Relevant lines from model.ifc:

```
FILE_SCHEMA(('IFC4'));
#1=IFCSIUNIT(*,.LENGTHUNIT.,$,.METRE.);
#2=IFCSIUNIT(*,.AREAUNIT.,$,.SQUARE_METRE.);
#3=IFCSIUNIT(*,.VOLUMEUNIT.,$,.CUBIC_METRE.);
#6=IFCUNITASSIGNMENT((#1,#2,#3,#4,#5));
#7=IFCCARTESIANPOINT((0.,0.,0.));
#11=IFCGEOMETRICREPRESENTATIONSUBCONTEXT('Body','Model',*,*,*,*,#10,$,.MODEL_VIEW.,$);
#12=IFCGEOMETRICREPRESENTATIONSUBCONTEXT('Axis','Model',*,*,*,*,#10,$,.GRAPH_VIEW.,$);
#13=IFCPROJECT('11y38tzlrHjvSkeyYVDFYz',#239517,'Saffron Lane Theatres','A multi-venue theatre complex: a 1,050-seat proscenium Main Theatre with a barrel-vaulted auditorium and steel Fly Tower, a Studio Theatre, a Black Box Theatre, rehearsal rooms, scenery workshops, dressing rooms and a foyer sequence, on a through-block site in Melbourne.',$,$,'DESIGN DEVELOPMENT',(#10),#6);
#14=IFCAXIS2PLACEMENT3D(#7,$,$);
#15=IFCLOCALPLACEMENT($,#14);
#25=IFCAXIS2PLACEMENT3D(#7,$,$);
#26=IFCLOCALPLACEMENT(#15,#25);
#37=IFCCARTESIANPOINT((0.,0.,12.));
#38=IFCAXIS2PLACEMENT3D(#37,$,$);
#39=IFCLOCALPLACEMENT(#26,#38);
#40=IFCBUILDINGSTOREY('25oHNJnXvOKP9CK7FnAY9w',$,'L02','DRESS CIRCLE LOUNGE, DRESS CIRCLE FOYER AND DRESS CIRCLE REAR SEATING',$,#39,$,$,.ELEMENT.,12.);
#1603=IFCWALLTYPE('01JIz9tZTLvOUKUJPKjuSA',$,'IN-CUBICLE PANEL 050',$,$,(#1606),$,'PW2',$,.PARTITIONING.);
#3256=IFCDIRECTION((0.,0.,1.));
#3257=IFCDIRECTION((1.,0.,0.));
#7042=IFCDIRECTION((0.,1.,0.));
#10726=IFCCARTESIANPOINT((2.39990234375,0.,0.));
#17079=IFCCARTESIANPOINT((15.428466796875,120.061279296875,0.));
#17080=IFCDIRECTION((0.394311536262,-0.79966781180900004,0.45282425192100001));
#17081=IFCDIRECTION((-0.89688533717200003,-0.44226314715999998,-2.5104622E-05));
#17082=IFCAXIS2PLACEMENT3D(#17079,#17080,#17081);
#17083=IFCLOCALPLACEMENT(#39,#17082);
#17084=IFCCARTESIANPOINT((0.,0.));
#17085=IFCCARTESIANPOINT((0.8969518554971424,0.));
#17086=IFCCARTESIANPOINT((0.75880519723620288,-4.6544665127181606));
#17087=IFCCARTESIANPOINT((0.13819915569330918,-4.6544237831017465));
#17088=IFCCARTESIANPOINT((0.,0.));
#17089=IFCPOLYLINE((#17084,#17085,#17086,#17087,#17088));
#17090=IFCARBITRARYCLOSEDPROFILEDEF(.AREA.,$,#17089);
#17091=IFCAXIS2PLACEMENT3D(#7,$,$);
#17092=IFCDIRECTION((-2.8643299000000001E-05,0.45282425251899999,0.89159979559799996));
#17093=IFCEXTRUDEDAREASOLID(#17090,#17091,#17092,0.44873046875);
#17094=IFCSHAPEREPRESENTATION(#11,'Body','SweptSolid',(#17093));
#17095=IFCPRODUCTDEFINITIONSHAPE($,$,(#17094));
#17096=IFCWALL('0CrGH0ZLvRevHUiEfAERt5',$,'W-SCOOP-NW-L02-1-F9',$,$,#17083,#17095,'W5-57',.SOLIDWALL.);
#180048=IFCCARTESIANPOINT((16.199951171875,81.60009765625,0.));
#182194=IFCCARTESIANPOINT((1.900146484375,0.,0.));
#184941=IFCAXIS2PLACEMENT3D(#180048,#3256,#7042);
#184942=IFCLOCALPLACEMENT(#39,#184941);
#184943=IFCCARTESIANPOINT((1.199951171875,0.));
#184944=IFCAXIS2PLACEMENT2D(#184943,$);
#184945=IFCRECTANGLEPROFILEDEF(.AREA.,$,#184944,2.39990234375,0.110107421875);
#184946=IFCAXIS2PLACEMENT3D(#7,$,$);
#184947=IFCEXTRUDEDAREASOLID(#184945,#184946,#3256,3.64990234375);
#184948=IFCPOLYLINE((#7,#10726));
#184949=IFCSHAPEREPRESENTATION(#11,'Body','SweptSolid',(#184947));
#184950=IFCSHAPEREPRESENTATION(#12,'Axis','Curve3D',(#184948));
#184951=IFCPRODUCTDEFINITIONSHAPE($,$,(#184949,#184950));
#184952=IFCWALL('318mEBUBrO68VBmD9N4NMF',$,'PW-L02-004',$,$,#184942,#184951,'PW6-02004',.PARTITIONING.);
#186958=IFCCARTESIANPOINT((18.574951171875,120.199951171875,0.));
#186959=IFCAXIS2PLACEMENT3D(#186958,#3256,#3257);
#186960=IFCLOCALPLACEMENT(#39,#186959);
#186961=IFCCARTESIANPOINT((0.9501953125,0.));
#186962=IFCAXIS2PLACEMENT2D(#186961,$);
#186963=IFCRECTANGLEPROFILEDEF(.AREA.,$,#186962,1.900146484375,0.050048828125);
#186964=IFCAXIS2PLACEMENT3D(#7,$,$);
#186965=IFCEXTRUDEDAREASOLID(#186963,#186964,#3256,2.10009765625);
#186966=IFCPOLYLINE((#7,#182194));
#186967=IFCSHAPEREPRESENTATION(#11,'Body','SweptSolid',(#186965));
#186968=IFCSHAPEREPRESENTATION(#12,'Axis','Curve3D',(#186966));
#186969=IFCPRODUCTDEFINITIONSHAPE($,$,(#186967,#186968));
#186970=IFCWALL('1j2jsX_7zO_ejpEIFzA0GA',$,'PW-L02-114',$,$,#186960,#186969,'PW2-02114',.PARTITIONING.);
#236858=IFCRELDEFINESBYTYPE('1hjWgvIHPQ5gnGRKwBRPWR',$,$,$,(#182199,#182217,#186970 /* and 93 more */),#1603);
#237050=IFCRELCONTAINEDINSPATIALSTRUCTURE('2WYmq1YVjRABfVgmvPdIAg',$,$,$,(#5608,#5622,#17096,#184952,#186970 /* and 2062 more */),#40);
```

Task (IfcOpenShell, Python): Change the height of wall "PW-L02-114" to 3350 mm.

```python
import ifcopenshell
import ifcopenshell.geom
import ifcopenshell.util.representation
import ifcopenshell.util.shape
import ifcopenshell.util.unit

model = ifcopenshell.open("model.ifc")
unit_scale = ifcopenshell.util.unit.calculate_unit_scale(model)
settings = ifcopenshell.geom.settings()


def volume(element):
    """Net volume in cubic metres, openings subtracted."""
    shape = ifcopenshell.geom.create_shape(settings, element)
    return ifcopenshell.util.shape.get_volume(shape.geometry)


wall = model.by_id(186970)
before = volume(wall)

body = ifcopenshell.util.representation.get_representation(wall, "Model", "Body")
solid = body.Items[0]
old_height = solid.Depth
solid.Depth = 3.35 / unit_scale
after = volume(wall)

print(f"height {old_height:g} -> {solid.Depth:g}, volume {before:.3f} -> {after:.3f} m3")

model.write("model_edited.ifc")
```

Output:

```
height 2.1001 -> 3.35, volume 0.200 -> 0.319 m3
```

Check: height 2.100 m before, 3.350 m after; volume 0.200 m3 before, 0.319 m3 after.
